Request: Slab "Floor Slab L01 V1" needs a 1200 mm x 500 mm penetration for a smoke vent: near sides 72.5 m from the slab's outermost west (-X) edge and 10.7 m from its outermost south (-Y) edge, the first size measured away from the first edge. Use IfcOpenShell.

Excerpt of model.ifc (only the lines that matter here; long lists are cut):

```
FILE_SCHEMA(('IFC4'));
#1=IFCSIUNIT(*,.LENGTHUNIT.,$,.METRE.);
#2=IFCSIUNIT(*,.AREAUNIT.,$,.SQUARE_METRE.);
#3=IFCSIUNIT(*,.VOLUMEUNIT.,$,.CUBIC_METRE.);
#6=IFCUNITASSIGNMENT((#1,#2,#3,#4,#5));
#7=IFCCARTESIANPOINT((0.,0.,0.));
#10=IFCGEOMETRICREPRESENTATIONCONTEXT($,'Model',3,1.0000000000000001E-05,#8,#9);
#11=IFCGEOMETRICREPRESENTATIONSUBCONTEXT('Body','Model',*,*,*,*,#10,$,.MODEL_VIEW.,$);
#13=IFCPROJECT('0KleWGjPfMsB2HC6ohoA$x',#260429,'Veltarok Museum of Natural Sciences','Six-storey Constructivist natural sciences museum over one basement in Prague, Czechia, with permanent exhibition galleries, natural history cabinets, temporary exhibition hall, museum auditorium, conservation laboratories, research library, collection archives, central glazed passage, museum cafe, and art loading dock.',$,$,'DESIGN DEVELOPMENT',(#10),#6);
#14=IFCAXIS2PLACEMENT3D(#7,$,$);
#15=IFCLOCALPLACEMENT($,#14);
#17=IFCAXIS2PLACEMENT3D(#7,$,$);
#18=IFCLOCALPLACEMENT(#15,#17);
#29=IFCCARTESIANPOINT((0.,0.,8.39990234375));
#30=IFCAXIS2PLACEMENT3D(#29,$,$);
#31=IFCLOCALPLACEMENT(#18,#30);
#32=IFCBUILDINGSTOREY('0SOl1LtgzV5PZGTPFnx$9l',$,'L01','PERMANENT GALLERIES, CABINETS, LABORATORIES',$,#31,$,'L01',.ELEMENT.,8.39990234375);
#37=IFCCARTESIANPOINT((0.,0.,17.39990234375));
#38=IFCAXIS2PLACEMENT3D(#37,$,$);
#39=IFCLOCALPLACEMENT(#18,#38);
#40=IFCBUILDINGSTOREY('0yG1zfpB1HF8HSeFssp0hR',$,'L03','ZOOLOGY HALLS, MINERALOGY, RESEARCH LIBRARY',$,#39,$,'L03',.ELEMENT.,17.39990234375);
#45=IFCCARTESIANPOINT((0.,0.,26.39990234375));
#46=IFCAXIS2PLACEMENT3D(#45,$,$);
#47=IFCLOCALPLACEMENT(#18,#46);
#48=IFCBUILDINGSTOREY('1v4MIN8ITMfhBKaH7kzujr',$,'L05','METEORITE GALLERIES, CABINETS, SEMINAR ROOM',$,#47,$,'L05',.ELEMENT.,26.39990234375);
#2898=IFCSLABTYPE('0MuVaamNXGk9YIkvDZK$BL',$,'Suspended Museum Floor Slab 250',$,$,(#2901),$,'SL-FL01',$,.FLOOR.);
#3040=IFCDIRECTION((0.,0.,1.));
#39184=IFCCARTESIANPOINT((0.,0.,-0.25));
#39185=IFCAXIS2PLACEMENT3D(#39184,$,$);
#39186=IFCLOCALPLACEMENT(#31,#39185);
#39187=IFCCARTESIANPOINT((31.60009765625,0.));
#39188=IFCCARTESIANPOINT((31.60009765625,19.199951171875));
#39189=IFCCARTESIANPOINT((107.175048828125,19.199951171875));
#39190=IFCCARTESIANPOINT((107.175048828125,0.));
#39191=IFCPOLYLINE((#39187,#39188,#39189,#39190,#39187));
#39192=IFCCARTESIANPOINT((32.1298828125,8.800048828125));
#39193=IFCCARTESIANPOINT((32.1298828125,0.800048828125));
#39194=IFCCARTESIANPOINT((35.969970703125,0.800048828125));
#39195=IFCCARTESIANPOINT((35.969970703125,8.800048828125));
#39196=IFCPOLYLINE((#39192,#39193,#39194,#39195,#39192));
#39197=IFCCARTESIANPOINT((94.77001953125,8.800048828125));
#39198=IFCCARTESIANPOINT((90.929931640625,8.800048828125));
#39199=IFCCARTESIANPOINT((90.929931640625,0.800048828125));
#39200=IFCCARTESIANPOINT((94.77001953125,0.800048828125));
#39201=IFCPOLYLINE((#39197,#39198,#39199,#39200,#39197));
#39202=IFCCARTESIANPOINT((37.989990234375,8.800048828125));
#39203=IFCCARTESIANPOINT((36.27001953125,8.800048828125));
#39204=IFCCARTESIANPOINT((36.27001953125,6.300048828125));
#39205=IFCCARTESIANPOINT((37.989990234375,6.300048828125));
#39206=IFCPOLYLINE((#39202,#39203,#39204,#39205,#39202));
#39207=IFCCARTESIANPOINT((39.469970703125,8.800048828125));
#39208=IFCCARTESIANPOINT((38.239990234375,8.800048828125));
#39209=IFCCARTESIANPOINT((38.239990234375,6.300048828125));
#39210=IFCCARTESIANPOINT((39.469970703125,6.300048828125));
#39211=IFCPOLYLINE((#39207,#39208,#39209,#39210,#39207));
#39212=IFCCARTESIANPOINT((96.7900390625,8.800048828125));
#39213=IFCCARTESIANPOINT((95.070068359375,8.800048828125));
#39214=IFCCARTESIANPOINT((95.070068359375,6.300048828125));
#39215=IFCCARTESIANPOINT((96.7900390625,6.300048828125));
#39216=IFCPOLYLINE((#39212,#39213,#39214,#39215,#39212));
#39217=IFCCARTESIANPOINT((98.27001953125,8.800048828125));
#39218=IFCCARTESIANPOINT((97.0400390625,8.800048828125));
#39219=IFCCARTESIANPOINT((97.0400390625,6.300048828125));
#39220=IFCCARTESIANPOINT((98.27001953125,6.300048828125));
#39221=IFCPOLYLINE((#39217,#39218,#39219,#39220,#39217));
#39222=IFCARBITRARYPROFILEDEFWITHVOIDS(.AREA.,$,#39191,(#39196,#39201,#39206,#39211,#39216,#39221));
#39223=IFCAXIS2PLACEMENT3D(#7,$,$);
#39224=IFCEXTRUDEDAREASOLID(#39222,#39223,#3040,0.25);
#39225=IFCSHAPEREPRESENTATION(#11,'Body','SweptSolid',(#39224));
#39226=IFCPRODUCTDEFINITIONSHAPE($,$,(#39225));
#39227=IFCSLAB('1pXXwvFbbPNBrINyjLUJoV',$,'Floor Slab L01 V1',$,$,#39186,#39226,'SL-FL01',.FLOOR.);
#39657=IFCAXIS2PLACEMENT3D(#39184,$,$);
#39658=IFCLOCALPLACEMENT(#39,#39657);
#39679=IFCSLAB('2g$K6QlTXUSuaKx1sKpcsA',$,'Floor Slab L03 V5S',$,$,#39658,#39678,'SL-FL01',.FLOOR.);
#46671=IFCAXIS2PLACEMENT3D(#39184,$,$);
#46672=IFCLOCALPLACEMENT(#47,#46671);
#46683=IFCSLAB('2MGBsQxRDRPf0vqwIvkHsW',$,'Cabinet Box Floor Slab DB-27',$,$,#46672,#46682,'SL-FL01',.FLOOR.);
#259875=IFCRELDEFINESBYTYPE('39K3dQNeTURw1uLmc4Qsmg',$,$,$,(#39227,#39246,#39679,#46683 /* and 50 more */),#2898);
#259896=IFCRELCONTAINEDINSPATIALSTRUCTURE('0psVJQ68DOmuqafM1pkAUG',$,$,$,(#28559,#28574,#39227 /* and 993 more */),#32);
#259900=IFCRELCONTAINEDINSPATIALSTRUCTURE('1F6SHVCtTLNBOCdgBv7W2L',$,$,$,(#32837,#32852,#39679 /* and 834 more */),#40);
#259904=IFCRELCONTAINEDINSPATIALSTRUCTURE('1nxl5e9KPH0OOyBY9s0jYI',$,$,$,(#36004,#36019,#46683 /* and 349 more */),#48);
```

```python
import numpy as np
import ifcopenshell
import ifcopenshell.api.feature
import ifcopenshell.api.geometry
import ifcopenshell.api.root
import ifcopenshell.geom
import ifcopenshell.util.placement
import ifcopenshell.util.representation
import ifcopenshell.util.shape
import ifcopenshell.util.unit

model = ifcopenshell.open("model.ifc")
unit_scale = ifcopenshell.util.unit.calculate_unit_scale(model)
settings = ifcopenshell.geom.settings()


def volume(element):
    """Net volume in cubic metres, openings subtracted."""
    shape = ifcopenshell.geom.create_shape(settings, element)
    return ifcopenshell.util.shape.get_volume(shape.geometry)


slab = model.by_id(39227)
before = volume(slab)

# Extent in the slab's own axes, in metres. The edges named are its -X and -Y sides.
slab_shape = ifcopenshell.geom.create_shape(settings, slab)
vertices = ifcopenshell.util.shape.get_vertices(slab_shape.geometry)
x_min, y_min, bottom = vertices.min(axis=0)
top = vertices[:, 2].max()

opening = ifcopenshell.api.root.create_entity(model, ifc_class="IfcOpeningElement", name="Smoke vent opening", predefined_type="OPENING")
context = ifcopenshell.util.representation.get_context(model, "Model", "Body", "MODEL_VIEW")
width, depth = 1.2, 0.5
outline = [(0.0, 0.0), (width, 0.0), (width, depth), (0.0, depth), (0.0, 0.0)]
# Overshoot both faces by 50 mm so the cut is clean.
shape = ifcopenshell.api.geometry.add_slab_representation(
    model, context=context, depth=top - bottom + 0.1, polyline=outline
)
ifcopenshell.api.geometry.assign_representation(model, product=opening, representation=shape)

matrix = ifcopenshell.util.placement.get_local_placement(slab.ObjectPlacement)
matrix[:, 3] = matrix @ np.append(np.array([x_min + 72.5, y_min + 10.7, bottom - 0.05]) / unit_scale, 1.0)
ifcopenshell.api.geometry.edit_object_placement(model, product=opening, matrix=matrix, is_si=False)
ifcopenshell.api.feature.add_feature(model, feature=opening, element=slab)

after = volume(slab)

print(f"slab volume {before:.3f} -> {after:.3f} m3")

model.write("model_edited.ifc")
```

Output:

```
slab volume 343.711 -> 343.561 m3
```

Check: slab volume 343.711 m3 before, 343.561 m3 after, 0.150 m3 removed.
